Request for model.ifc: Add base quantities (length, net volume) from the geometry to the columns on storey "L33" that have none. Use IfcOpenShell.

First a look at what the model holds.

```python
import ifcopenshell
import ifcopenshell.util.element
import ifcopenshell.util.unit

model = ifcopenshell.open("model.ifc")
print(model.schema)
for unit_type in ("LENGTHUNIT", "AREAUNIT", "VOLUMEUNIT"):
    print(unit_type, ifcopenshell.util.unit.calculate_unit_scale(model, unit_type))
storey = next(s for s in model.by_type("IfcBuildingStorey") if s.Name == "L33")
columns = [e for e in ifcopenshell.util.element.get_decomposition(storey) if e.is_a("IfcColumn")]
for e in sorted(columns, key=lambda e: e.id()):
    print(e.id(), e.is_a(), e.Name, list(ifcopenshell.util.element.get_psets(e, qtos_only=True)), sep=" | ")
```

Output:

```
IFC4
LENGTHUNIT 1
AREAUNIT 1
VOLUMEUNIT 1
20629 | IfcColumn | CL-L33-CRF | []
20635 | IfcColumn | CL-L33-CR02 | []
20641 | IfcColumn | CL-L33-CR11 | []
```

```python
import ifcopenshell
import ifcopenshell.api.pset
import ifcopenshell.geom
import ifcopenshell.util.element
import ifcopenshell.util.shape
import ifcopenshell.util.unit

model = ifcopenshell.open("model.ifc")
unit_scale = ifcopenshell.util.unit.calculate_unit_scale(model)
volume_scale = ifcopenshell.util.unit.calculate_unit_scale(model, "VOLUMEUNIT")
settings = ifcopenshell.geom.settings()

storey = next(s for s in model.by_type("IfcBuildingStorey") if s.Name == "L33")
columns = [e for e in ifcopenshell.util.element.get_decomposition(storey) if e.is_a("IfcColumn")]

for e in sorted(columns, key=lambda e: e.id()):
    if ifcopenshell.util.element.get_psets(e, qtos_only=True, should_inherit=False):
        continue
    # Geometry comes back in metres, in the element's own axes.
    shape = ifcopenshell.geom.create_shape(settings, e)
    values = {
        "Length": ifcopenshell.util.shape.get_z(shape.geometry) / unit_scale,
        "NetVolume": ifcopenshell.util.shape.get_volume(shape.geometry) / volume_scale,
    }
    qto = ifcopenshell.api.pset.add_qto(model, product=e, name="Qto_ColumnBaseQuantities")
    ifcopenshell.api.pset.edit_qto(model, qto=qto, properties=values)
    print(e.id(), {k: round(v, 3) for k, v in values.items()})

model.write("model_v2.ifc")
```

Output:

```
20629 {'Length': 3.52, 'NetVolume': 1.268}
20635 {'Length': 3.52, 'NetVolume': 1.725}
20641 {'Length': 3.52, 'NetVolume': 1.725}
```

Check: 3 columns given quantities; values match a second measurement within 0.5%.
